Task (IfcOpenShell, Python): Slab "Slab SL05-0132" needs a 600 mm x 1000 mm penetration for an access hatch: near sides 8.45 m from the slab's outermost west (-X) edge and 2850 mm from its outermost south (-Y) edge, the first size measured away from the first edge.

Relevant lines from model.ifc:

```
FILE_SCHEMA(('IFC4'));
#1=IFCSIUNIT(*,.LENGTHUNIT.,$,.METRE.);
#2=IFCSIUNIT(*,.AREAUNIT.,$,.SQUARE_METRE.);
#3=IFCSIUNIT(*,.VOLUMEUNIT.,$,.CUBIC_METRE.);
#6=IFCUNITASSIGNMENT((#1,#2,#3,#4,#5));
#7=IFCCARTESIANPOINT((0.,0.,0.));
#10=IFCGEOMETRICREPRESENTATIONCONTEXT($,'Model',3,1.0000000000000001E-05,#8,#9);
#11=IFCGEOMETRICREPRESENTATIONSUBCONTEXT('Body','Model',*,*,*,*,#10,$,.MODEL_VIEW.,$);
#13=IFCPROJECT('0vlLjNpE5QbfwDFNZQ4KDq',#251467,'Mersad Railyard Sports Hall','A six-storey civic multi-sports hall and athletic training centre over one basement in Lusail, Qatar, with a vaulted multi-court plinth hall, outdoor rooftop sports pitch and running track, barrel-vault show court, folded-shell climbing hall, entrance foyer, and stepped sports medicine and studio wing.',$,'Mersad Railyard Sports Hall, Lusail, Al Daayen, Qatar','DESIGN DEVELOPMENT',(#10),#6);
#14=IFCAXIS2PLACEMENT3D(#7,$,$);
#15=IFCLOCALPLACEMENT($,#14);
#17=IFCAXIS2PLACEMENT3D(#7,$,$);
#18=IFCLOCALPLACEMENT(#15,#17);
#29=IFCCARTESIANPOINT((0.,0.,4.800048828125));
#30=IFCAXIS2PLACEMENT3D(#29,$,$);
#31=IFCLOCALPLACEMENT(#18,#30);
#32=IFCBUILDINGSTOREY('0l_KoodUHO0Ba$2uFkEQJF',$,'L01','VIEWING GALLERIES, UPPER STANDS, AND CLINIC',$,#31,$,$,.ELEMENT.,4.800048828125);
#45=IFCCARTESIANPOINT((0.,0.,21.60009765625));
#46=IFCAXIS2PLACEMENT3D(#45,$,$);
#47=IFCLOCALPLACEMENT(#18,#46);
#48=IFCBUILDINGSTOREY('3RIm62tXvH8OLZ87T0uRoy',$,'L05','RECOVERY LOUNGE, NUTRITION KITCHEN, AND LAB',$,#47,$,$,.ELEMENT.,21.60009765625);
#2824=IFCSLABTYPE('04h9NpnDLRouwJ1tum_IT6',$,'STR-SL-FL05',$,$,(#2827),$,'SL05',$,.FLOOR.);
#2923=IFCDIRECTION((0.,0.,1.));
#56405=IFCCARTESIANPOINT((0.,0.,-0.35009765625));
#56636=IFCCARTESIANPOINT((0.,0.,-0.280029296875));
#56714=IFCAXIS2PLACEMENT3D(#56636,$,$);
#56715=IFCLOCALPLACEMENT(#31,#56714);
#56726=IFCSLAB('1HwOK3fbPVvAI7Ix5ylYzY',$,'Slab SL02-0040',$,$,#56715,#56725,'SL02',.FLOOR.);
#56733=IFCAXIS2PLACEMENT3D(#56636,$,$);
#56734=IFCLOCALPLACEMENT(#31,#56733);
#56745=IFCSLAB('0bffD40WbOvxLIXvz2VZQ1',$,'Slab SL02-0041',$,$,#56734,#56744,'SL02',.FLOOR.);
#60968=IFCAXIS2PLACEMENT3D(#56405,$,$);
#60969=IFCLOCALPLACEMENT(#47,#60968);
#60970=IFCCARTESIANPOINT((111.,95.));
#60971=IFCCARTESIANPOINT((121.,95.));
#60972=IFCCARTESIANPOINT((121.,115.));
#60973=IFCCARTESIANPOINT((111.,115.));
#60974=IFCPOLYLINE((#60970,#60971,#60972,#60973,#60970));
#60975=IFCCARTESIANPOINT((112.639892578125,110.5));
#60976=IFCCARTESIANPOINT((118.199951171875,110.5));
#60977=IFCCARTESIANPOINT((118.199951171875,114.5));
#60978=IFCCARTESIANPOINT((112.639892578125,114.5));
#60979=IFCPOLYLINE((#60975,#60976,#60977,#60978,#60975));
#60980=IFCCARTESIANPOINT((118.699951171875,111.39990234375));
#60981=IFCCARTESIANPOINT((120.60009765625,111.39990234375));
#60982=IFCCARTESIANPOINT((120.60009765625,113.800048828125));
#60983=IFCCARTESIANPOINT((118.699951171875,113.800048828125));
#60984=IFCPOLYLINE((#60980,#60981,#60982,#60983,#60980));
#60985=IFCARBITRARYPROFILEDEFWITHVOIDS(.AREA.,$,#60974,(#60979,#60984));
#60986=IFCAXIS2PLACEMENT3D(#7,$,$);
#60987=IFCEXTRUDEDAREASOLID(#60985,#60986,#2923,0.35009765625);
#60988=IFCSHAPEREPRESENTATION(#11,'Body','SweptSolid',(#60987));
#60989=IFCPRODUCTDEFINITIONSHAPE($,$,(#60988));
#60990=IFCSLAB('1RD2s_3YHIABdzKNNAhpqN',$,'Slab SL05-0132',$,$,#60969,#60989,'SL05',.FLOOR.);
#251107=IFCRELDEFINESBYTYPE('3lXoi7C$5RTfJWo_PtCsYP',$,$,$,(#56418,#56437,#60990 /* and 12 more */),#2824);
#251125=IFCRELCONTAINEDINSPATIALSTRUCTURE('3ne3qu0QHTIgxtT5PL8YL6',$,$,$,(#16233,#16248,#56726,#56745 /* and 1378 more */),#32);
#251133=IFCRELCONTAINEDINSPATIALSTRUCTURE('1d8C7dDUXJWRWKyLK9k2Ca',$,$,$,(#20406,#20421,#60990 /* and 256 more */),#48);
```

```python
import numpy as np
import ifcopenshell
import ifcopenshell.api.feature
import ifcopenshell.api.geometry
import ifcopenshell.api.root
import ifcopenshell.geom
import ifcopenshell.util.placement
import ifcopenshell.util.representation
import ifcopenshell.util.shape
import ifcopenshell.util.unit

model = ifcopenshell.open("model.ifc")
unit_scale = ifcopenshell.util.unit.calculate_unit_scale(model)
settings = ifcopenshell.geom.settings()


def volume(element):
    """Net volume in cubic metres, openings subtracted."""
    shape = ifcopenshell.geom.create_shape(settings, element)
    return ifcopenshell.util.shape.get_volume(shape.geometry)


slab = model.by_guid("1RD2s_3YHIABdzKNNAhpqN")
before = volume(slab)

# Extent in the slab's own axes, in metres. The edges named are its -X and -Y sides.
slab_shape = ifcopenshell.geom.create_shape(settings, slab)
vertices = ifcopenshell.util.shape.get_vertices(slab_shape.geometry)
x_min, y_min, bottom = vertices.min(axis=0)
top = vertices[:, 2].max()

opening = ifcopenshell.api.root.create_entity(model, ifc_class="IfcOpeningElement", name="Access hatch opening", predefined_type="OPENING")
context = ifcopenshell.util.representation.get_context(model, "Model", "Body", "MODEL_VIEW")
width, depth = 0.6, 1
outline = [(0.0, 0.0), (width, 0.0), (width, depth), (0.0, depth), (0.0, 0.0)]
# Overshoot both faces by 50 mm so the cut is clean.
shape = ifcopenshell.api.geometry.add_slab_representation(
    model, context=context, depth=top - bottom + 0.1, polyline=outline
)
ifcopenshell.api.geometry.assign_representation(model, product=opening, representation=shape)

matrix = ifcopenshell.util.placement.get_local_placement(slab.ObjectPlacement)
matrix[:, 3] = matrix @ np.append(np.array([x_min + 8.45, y_min + 2.85, bottom - 0.05]) / unit_scale, 1.0)
ifcopenshell.api.geometry.edit_object_placement(model, product=opening, matrix=matrix, is_si=False)
ifcopenshell.api.feature.add_feature(model, feature=opening, element=slab)

after = volume(slab)

print(f"slab volume {before:.3f} -> {after:.3f} m3")

model.write("model_updated.ifc")
```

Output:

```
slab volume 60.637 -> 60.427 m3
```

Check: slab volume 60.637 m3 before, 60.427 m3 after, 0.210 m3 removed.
